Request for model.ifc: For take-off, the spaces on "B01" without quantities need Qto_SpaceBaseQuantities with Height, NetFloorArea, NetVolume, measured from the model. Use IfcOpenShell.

First a look at what the model holds.

```python
import ifcopenshell
import ifcopenshell.util.element
import ifcopenshell.util.unit

model = ifcopenshell.open("model.ifc")
print(model.schema)
for unit_type in ("LENGTHUNIT", "AREAUNIT", "VOLUMEUNIT"):
    print(unit_type, ifcopenshell.util.unit.calculate_unit_scale(model, unit_type))
storey = next(s for s in model.by_type("IfcBuildingStorey") if s.Name == "B01")
spaces = [e for e in ifcopenshell.util.element.get_decomposition(storey) if e.is_a("IfcSpace")]
for e in sorted(spaces, key=lambda e: e.id()):
    print(e.id(), e.is_a(), e.Name, list(ifcopenshell.util.element.get_psets(e, qtos_only=True)), sep=" | ")
```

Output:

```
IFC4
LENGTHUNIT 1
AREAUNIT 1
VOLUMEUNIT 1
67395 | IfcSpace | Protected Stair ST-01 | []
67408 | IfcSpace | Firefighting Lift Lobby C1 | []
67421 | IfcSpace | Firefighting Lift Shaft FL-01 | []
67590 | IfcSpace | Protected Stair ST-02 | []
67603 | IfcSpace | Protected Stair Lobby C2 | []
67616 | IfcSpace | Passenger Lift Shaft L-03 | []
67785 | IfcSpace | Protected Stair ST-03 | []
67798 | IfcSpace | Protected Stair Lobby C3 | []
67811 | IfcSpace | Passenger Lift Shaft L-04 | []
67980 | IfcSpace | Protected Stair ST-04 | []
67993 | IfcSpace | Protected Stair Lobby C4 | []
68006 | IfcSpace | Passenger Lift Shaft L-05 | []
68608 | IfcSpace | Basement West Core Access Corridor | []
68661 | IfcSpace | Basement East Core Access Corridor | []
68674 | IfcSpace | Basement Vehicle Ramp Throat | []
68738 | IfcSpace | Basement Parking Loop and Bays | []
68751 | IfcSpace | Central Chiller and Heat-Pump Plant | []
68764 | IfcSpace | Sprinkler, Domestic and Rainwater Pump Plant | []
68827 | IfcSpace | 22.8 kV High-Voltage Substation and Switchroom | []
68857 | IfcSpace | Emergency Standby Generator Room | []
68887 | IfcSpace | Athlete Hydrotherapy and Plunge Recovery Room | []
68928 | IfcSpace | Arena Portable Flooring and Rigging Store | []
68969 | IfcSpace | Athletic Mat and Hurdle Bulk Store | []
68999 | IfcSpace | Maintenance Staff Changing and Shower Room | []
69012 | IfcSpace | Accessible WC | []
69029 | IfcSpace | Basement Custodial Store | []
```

```python
import ifcopenshell
import ifcopenshell.api.pset
import ifcopenshell.geom
import ifcopenshell.util.element
import ifcopenshell.util.shape
import ifcopenshell.util.unit

model = ifcopenshell.open("model.ifc")
unit_scale = ifcopenshell.util.unit.calculate_unit_scale(model)
area_scale = ifcopenshell.util.unit.calculate_unit_scale(model, "AREAUNIT")
volume_scale = ifcopenshell.util.unit.calculate_unit_scale(model, "VOLUMEUNIT")
settings = ifcopenshell.geom.settings()

storey = next(s for s in model.by_type("IfcBuildingStorey") if s.Name == "B01")
spaces = [e for e in ifcopenshell.util.element.get_decomposition(storey) if e.is_a("IfcSpace")]

for e in sorted(spaces, key=lambda e: e.id()):
    if ifcopenshell.util.element.get_psets(e, qtos_only=True, should_inherit=False):
        continue
    # Geometry comes back in metres, in the element's own axes.
    shape = ifcopenshell.geom.create_shape(settings, e)
    values = {
        "Height": ifcopenshell.util.shape.get_z(shape.geometry) / unit_scale,
        "NetFloorArea": ifcopenshell.util.shape.get_footprint_area(shape.geometry) / area_scale,
        "NetVolume": ifcopenshell.util.shape.get_volume(shape.geometry) / volume_scale,
    }
    qto = ifcopenshell.api.pset.add_qto(model, product=e, name="Qto_SpaceBaseQuantities")
    ifcopenshell.api.pset.edit_qto(model, qto=qto, properties=values)
    print(e.id(), {k: round(v, 3) for k, v in values.items()})

model.write("model-out.ifc")
```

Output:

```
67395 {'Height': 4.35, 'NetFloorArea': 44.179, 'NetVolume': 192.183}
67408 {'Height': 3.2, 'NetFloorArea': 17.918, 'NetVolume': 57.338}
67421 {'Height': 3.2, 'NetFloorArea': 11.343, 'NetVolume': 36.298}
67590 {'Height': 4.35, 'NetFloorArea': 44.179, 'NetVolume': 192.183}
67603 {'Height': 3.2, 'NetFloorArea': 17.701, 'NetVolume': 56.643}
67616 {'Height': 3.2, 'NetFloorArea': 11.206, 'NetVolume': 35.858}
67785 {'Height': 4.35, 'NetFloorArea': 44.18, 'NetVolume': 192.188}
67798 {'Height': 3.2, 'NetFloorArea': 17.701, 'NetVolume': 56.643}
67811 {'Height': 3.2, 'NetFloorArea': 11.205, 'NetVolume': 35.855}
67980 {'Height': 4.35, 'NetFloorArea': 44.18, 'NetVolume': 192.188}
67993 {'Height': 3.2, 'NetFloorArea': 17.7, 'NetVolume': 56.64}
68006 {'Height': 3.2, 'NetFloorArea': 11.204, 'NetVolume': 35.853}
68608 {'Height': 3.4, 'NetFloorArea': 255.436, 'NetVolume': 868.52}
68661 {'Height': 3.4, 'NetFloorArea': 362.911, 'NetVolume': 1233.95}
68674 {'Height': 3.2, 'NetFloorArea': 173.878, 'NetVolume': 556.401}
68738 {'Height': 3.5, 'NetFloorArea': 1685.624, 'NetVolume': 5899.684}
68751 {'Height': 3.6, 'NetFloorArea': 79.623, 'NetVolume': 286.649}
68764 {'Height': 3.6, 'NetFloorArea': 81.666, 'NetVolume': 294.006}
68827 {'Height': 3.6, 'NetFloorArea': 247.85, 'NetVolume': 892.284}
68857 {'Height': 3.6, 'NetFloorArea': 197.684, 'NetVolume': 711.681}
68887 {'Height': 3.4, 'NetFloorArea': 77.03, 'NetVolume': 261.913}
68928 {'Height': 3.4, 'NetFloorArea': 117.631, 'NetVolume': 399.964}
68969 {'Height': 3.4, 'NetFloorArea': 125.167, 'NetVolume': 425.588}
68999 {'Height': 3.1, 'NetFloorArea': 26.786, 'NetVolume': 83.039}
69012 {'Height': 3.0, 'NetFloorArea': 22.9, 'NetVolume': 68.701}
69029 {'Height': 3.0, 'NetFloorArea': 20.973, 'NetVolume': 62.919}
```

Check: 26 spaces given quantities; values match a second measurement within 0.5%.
